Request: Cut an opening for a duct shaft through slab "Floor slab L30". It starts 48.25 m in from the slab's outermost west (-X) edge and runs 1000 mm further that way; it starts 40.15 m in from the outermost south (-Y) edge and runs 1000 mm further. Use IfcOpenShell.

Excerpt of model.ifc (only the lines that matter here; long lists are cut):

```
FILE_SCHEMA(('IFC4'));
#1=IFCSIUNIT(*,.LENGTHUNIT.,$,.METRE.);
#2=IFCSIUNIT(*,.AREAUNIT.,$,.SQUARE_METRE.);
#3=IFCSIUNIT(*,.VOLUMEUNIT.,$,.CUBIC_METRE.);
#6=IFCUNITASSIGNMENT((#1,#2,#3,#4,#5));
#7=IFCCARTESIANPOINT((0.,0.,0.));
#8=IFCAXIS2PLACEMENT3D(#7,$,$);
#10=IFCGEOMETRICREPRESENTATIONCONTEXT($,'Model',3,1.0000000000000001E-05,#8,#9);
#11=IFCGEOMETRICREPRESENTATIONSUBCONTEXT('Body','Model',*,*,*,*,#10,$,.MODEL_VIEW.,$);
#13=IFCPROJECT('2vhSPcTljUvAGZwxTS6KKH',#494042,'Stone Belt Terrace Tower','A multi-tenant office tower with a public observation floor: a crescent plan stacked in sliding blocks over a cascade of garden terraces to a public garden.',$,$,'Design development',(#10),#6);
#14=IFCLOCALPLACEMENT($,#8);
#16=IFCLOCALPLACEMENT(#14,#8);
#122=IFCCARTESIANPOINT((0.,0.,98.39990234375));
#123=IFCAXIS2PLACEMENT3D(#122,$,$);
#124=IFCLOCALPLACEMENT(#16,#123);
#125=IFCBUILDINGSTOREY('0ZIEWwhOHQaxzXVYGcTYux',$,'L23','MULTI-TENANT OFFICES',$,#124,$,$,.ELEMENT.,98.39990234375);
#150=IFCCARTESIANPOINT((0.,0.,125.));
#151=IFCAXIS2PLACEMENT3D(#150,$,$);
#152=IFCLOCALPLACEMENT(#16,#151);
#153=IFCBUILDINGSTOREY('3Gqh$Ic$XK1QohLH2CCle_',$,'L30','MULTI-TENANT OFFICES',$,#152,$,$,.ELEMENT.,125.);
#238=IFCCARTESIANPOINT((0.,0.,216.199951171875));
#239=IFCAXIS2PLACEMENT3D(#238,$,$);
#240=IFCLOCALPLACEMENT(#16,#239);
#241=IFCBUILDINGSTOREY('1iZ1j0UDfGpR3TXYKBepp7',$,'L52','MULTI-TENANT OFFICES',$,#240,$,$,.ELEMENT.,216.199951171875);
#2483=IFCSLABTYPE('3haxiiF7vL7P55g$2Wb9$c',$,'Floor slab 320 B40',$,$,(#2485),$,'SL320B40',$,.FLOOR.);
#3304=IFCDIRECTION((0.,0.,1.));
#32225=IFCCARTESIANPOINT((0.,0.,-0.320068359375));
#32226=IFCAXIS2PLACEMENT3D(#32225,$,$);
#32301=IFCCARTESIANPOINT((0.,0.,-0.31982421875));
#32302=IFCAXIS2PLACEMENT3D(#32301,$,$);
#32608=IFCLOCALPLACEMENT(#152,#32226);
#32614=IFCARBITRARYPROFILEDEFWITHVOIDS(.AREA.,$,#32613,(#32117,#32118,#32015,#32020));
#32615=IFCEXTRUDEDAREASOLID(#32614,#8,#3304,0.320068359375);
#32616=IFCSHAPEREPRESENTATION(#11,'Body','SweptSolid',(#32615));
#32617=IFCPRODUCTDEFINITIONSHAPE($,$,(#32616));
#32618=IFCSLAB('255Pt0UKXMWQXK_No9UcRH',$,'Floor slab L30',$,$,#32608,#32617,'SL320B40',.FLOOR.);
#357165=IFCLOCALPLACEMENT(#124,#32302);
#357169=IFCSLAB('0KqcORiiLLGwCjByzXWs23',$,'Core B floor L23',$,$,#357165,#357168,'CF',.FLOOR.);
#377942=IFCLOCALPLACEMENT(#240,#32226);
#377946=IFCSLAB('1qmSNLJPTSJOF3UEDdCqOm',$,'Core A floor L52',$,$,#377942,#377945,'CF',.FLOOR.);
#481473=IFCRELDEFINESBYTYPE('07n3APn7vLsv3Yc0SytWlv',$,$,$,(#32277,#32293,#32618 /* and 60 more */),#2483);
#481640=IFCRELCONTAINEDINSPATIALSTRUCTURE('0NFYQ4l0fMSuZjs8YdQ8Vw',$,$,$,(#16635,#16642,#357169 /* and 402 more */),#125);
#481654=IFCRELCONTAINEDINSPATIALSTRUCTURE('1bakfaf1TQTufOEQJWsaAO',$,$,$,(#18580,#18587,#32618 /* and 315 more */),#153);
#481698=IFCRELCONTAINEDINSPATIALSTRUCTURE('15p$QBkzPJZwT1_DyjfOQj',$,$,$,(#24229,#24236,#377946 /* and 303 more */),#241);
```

```python
import numpy as np
import ifcopenshell
import ifcopenshell.api.feature
import ifcopenshell.api.geometry
import ifcopenshell.api.root
import ifcopenshell.geom
import ifcopenshell.util.placement
import ifcopenshell.util.representation
import ifcopenshell.util.shape
import ifcopenshell.util.unit

model = ifcopenshell.open("model.ifc")
unit_scale = ifcopenshell.util.unit.calculate_unit_scale(model)
settings = ifcopenshell.geom.settings()


def volume(element):
    """Net volume in cubic metres, openings subtracted."""
    shape = ifcopenshell.geom.create_shape(settings, element)
    return ifcopenshell.util.shape.get_volume(shape.geometry)


slab = model.by_id(32618)
before = volume(slab)

# Extent in the slab's own axes, in metres. The edges named are its -X and -Y sides.
slab_shape = ifcopenshell.geom.create_shape(settings, slab)
vertices = ifcopenshell.util.shape.get_vertices(slab_shape.geometry)
x_min, y_min, bottom = vertices.min(axis=0)
top = vertices[:, 2].max()

opening = ifcopenshell.api.root.create_entity(model, ifc_class="IfcOpeningElement", name="Duct shaft opening", predefined_type="OPENING")
context = ifcopenshell.util.representation.get_context(model, "Model", "Body", "MODEL_VIEW")
width, depth = 1, 1
outline = [(0.0, 0.0), (width, 0.0), (width, depth), (0.0, depth), (0.0, 0.0)]
# Overshoot both faces by 50 mm so the cut is clean.
shape = ifcopenshell.api.geometry.add_slab_representation(
    model, context=context, depth=top - bottom + 0.1, polyline=outline
)
ifcopenshell.api.geometry.assign_representation(model, product=opening, representation=shape)

matrix = ifcopenshell.util.placement.get_local_placement(slab.ObjectPlacement)
matrix[:, 3] = matrix @ np.append(np.array([x_min + 48.25, y_min + 40.15, bottom - 0.05]) / unit_scale, 1.0)
ifcopenshell.api.geometry.edit_object_placement(model, product=opening, matrix=matrix, is_si=False)
ifcopenshell.api.feature.add_feature(model, feature=opening, element=slab)

after = volume(slab)

print(f"slab volume {before:.3f} -> {after:.3f} m3")

model.write("model_v2.ifc")
```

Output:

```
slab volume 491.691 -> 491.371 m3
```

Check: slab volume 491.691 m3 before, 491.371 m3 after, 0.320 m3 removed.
